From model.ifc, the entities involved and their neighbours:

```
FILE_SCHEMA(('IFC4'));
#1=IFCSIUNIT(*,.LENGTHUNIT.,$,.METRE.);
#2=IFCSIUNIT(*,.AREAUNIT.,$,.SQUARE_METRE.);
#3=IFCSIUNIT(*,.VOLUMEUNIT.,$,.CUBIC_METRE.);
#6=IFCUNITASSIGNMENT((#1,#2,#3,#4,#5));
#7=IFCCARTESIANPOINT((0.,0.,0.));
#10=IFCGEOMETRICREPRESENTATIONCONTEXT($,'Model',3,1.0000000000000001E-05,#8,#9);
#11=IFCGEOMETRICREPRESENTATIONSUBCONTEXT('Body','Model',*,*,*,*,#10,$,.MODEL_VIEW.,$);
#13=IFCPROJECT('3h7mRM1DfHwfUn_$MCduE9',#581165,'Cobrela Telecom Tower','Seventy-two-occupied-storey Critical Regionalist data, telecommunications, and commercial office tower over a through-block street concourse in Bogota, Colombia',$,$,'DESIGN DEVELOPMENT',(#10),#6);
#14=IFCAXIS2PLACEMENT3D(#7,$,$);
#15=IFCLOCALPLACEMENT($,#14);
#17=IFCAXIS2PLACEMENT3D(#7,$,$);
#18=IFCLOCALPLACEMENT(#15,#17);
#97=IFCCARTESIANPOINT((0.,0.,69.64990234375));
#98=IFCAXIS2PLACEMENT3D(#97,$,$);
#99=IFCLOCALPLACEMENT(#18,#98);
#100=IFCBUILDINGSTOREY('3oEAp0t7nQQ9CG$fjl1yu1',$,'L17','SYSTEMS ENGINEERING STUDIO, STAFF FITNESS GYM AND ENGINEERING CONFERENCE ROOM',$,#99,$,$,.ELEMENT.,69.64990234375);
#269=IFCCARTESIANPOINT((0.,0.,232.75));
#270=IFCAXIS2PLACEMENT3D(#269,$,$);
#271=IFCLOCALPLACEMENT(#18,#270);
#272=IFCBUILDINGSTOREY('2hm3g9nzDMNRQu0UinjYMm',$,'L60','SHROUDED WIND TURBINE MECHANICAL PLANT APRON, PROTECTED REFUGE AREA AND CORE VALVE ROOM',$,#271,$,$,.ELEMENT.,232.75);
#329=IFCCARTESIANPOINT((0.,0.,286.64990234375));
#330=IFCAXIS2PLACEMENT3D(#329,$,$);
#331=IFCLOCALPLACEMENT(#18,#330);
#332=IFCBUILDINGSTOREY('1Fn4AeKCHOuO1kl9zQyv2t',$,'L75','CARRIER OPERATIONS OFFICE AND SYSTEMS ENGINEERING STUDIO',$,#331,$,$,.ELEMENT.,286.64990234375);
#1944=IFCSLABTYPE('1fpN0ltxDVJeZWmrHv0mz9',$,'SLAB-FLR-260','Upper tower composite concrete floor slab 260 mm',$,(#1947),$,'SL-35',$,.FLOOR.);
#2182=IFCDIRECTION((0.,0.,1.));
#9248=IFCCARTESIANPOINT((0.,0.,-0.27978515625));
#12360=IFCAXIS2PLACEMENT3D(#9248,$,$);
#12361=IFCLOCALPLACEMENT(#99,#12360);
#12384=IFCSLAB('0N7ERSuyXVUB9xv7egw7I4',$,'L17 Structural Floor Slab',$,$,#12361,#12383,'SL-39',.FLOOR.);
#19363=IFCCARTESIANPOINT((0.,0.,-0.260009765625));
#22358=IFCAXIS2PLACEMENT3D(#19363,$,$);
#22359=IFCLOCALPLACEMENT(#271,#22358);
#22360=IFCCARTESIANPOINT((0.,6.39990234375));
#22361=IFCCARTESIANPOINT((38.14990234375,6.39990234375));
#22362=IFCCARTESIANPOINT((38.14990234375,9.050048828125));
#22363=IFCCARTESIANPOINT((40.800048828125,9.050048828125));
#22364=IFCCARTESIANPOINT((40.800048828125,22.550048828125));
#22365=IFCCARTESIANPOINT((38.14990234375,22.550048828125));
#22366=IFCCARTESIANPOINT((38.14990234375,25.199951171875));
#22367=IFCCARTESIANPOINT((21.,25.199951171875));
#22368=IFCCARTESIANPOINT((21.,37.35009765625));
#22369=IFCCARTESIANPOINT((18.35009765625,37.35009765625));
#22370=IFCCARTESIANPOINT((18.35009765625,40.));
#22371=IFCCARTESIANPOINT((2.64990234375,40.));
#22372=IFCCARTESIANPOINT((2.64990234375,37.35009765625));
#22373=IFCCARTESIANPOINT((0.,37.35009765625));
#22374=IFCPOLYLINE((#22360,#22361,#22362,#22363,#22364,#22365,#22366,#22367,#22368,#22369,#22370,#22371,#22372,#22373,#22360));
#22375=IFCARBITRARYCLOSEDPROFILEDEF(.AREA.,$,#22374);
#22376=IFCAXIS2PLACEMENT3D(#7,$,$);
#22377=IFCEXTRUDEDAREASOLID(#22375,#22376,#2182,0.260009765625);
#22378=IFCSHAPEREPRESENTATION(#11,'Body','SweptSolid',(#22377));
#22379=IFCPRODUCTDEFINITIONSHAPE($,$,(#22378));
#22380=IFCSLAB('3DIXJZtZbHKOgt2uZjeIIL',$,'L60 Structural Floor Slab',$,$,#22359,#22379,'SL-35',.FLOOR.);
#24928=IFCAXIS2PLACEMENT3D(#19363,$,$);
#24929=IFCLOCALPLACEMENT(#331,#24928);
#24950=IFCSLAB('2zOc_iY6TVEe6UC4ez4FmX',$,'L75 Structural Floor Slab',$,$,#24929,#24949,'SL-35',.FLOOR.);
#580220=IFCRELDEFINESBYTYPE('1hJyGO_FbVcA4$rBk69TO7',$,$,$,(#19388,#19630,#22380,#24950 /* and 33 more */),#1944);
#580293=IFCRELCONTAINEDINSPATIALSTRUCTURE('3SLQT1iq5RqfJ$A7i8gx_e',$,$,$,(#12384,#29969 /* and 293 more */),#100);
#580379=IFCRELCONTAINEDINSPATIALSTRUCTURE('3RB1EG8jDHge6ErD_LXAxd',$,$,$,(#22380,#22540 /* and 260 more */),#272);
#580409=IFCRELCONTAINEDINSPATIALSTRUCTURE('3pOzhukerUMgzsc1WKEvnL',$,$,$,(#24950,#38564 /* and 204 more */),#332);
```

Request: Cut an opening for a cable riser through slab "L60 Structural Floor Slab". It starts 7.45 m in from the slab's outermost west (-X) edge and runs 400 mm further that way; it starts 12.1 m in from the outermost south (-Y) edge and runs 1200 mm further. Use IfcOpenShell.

```python
import numpy as np
import ifcopenshell
import ifcopenshell.api.feature
import ifcopenshell.api.geometry
import ifcopenshell.api.root
import ifcopenshell.geom
import ifcopenshell.util.placement
import ifcopenshell.util.representation
import ifcopenshell.util.shape
import ifcopenshell.util.unit

model = ifcopenshell.open("model.ifc")
unit_scale = ifcopenshell.util.unit.calculate_unit_scale(model)
settings = ifcopenshell.geom.settings()


def volume(element):
    """Net volume in cubic metres, openings subtracted."""
    shape = ifcopenshell.geom.create_shape(settings, element)
    return ifcopenshell.util.shape.get_volume(shape.geometry)


slab = model.by_id(22380)
before = volume(slab)

# Extent in the slab's own axes, in metres. The edges named are its -X and -Y sides.
slab_shape = ifcopenshell.geom.create_shape(settings, slab)
vertices = ifcopenshell.util.shape.get_vertices(slab_shape.geometry)
x_min, y_min, bottom = vertices.min(axis=0)
top = vertices[:, 2].max()

opening = ifcopenshell.api.root.create_entity(model, ifc_class="IfcOpeningElement", name="Cable riser opening", predefined_type="OPENING")
context = ifcopenshell.util.representation.get_context(model, "Model", "Body", "MODEL_VIEW")
width, depth = 0.4, 1.2
outline = [(0.0, 0.0), (width, 0.0), (width, depth), (0.0, depth), (0.0, 0.0)]
# Overshoot both faces by 50 mm so the cut is clean.
shape = ifcopenshell.api.geometry.add_slab_representation(
    model, context=context, depth=top - bottom + 0.1, polyline=outline
)
ifcopenshell.api.geometry.assign_representation(model, product=opening, representation=shape)

matrix = ifcopenshell.util.placement.get_local_placement(slab.ObjectPlacement)
matrix[:, 3] = matrix @ np.append(np.array([x_min + 7.45, y_min + 12.1, bottom - 0.05]) / unit_scale, 1.0)
ifcopenshell.api.geometry.edit_object_placement(model, product=opening, matrix=matrix, is_si=False)
ifcopenshell.api.feature.add_feature(model, feature=opening, element=slab)

after = volume(slab)

print(f"slab volume {before:.3f} -> {after:.3f} m3")

model.write("model_edited.ifc")
```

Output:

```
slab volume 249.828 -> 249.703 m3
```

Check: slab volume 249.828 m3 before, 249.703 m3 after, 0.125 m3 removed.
